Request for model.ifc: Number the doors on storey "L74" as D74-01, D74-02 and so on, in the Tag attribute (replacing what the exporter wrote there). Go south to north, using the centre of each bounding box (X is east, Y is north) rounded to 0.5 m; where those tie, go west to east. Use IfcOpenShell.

First a look at what the model holds.

```python
import ifcopenshell
import ifcopenshell.util.element
import ifcopenshell.util.placement

model = ifcopenshell.open("model.ifc")
print(model.schema)
storey = next(s for s in model.by_type("IfcBuildingStorey") if s.Name == "L74")
doors = [e for e in ifcopenshell.util.element.get_decomposition(storey) if e.is_a("IfcDoor")]
for e in sorted(doors, key=lambda e: e.id()):
    origin = ifcopenshell.util.placement.get_local_placement(e.ObjectPlacement)[:3, 3]
    print(e.id(), e.Tag, e.Name, origin.round(2) + 0.0, sep=" | ")
```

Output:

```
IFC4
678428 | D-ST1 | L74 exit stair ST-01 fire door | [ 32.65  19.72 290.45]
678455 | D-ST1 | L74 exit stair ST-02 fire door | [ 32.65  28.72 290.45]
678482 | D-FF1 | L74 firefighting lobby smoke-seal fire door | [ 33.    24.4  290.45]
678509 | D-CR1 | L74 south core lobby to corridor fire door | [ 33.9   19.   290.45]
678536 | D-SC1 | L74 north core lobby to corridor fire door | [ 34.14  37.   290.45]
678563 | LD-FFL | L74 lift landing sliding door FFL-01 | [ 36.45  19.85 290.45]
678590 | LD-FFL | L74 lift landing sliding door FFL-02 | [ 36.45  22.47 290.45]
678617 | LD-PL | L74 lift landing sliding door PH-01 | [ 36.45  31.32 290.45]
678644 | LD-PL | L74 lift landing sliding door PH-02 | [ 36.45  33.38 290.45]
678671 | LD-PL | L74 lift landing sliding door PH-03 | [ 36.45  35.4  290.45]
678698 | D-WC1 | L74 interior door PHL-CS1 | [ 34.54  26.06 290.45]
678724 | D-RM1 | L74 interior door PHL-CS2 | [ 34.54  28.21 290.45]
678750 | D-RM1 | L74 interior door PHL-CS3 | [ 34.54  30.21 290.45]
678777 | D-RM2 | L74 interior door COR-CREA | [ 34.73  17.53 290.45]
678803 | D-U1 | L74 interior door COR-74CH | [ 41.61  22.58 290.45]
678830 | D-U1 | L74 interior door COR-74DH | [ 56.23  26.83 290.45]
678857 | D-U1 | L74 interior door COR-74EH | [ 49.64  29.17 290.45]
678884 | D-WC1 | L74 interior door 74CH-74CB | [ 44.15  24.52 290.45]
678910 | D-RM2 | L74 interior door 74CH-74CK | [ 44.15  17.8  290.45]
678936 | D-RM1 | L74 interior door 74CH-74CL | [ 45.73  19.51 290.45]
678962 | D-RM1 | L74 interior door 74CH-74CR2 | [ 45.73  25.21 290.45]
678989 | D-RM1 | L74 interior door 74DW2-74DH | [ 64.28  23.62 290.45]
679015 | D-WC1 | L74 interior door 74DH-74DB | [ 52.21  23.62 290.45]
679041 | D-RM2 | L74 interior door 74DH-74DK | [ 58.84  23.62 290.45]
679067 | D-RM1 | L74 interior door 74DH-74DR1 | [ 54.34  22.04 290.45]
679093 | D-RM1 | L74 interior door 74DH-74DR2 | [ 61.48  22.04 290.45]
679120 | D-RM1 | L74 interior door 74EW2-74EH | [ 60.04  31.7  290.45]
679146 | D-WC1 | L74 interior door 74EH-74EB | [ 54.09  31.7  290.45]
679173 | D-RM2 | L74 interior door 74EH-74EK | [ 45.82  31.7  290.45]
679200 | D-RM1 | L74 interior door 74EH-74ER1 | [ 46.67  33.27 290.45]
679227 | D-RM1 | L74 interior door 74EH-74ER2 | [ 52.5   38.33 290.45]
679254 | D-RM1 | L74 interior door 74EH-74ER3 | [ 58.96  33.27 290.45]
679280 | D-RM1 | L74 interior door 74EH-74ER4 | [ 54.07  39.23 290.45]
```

```python
import ifcopenshell
import ifcopenshell.geom
import ifcopenshell.util.element
import ifcopenshell.util.shape

model = ifcopenshell.open("model.ifc")
settings = ifcopenshell.geom.settings()
settings.set("use-world-coords", True)


def centre(element):
    shape = ifcopenshell.geom.create_shape(settings, element)
    return ifcopenshell.util.shape.get_bbox_centroid(shape.geometry)


storey = next(s for s in model.by_type("IfcBuildingStorey") if s.Name == "L74")
doors = [e for e in ifcopenshell.util.element.get_decomposition(storey) if e.is_a("IfcDoor")]

# Insertion points can sit at a corner or the storey origin, so sort by the geometry (in metres).
centres = {e: centre(e) for e in doors}
doors.sort(key=lambda e: (round(centres[e][1] / 0.5), centres[e][0]))

for i, e in enumerate(doors, start=1):
    number = f"D74-{i:02d}"
    e.Tag = number
    print(e.id(), number)

model.write("model_v2.ifc")
```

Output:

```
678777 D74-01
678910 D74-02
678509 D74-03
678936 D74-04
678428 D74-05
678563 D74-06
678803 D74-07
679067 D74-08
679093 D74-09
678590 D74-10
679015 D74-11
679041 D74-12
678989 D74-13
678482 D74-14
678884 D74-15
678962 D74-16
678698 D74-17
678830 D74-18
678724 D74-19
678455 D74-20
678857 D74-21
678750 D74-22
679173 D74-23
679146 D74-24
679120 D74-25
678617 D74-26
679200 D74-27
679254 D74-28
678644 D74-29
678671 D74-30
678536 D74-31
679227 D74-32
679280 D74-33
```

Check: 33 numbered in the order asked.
